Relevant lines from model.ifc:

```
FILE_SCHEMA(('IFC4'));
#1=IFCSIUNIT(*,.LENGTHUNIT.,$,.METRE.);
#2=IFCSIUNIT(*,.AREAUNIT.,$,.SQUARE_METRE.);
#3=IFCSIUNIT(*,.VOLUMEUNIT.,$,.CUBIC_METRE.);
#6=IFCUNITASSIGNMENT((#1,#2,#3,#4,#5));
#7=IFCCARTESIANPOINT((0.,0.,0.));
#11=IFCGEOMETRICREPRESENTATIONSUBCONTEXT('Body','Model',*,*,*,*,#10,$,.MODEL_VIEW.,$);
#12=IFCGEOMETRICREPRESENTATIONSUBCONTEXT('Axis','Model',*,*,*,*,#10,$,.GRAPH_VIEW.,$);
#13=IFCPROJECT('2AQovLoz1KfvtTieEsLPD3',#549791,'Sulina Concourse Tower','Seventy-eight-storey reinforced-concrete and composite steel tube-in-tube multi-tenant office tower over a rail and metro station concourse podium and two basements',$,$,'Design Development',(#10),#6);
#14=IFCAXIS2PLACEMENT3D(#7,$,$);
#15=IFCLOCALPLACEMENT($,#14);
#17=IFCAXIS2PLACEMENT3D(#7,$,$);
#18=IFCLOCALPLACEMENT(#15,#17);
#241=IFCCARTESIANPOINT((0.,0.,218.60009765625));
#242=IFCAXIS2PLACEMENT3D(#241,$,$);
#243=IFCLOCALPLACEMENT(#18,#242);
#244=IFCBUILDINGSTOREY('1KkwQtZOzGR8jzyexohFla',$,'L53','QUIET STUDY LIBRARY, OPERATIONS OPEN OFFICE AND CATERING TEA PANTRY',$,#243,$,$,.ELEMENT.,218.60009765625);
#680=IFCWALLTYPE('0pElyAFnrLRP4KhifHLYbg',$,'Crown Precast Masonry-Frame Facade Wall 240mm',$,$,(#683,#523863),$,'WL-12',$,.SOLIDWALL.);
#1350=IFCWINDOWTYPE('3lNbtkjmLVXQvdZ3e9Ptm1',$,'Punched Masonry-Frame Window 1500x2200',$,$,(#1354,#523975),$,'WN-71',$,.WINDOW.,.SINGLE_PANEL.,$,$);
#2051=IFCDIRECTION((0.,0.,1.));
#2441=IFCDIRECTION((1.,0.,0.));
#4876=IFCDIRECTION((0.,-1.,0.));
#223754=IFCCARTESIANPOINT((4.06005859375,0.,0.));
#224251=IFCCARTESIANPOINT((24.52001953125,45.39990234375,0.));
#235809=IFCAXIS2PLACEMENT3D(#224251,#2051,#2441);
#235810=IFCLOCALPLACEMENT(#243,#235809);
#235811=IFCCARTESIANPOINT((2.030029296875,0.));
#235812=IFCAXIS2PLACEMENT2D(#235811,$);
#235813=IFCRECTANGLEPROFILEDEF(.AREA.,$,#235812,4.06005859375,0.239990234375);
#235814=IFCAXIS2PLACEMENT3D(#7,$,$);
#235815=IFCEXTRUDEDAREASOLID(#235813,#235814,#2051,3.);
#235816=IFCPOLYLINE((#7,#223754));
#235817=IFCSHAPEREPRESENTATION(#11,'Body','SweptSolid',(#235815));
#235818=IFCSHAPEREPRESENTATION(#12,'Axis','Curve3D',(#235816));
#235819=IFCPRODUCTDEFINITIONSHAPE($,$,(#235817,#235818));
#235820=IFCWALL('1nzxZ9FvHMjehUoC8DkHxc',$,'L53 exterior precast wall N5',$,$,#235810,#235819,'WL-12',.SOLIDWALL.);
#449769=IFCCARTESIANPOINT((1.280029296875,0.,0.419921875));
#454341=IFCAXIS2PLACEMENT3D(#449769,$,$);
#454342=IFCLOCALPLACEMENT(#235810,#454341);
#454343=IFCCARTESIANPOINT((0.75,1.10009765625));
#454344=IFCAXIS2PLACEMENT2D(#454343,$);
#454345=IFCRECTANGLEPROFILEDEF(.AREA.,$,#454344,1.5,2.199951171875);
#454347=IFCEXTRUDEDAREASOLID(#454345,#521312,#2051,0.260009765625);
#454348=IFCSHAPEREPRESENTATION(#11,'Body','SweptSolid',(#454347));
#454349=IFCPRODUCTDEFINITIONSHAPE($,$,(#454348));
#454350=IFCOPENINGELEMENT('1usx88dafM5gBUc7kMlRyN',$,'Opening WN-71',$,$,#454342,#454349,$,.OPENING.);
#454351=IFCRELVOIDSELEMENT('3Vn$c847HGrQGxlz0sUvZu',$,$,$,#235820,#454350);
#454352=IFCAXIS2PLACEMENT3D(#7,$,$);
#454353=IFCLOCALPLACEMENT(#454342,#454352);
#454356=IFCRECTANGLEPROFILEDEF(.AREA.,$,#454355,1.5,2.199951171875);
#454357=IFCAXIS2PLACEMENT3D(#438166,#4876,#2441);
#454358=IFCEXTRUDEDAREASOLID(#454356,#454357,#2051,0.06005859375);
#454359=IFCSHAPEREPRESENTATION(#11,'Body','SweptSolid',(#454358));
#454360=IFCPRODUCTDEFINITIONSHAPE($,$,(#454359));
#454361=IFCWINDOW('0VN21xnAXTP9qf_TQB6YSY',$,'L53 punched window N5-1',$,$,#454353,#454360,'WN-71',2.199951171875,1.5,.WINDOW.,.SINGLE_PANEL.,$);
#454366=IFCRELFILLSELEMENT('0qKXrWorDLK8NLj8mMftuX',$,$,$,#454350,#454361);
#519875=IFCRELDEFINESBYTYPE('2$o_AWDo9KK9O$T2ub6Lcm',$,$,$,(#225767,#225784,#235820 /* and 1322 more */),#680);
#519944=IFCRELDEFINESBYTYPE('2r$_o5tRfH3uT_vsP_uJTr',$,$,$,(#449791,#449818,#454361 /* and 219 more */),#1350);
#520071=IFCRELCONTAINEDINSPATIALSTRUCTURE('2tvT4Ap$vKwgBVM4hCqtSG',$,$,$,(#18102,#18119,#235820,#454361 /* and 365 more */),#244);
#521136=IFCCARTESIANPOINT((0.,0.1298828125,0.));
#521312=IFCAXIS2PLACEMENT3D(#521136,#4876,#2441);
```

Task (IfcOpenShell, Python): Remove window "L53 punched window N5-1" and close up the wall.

```python
import ifcopenshell
import ifcopenshell.api.feature
import ifcopenshell.api.root
import ifcopenshell.geom
import ifcopenshell.util.shape

model = ifcopenshell.open("model.ifc")
settings = ifcopenshell.geom.settings()


def volume(element):
    """Net volume in cubic metres, openings subtracted."""
    shape = ifcopenshell.geom.create_shape(settings, element)
    return ifcopenshell.util.shape.get_volume(shape.geometry)


window = model.by_guid("0VN21xnAXTP9qf_TQB6YSY")
opening = window.FillsVoids[0].RelatingOpeningElement
wall = opening.VoidsElements[0].RelatingBuildingElement
before = volume(wall)

ifcopenshell.api.root.remove_product(model, product=window)
ifcopenshell.api.feature.remove_feature(model, feature=opening)

after = volume(wall)

print(f"wall volume {before:.3f} -> {after:.3f} m3")

model.write("model_updated.ifc")
```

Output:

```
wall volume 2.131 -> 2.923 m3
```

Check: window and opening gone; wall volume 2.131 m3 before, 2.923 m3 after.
